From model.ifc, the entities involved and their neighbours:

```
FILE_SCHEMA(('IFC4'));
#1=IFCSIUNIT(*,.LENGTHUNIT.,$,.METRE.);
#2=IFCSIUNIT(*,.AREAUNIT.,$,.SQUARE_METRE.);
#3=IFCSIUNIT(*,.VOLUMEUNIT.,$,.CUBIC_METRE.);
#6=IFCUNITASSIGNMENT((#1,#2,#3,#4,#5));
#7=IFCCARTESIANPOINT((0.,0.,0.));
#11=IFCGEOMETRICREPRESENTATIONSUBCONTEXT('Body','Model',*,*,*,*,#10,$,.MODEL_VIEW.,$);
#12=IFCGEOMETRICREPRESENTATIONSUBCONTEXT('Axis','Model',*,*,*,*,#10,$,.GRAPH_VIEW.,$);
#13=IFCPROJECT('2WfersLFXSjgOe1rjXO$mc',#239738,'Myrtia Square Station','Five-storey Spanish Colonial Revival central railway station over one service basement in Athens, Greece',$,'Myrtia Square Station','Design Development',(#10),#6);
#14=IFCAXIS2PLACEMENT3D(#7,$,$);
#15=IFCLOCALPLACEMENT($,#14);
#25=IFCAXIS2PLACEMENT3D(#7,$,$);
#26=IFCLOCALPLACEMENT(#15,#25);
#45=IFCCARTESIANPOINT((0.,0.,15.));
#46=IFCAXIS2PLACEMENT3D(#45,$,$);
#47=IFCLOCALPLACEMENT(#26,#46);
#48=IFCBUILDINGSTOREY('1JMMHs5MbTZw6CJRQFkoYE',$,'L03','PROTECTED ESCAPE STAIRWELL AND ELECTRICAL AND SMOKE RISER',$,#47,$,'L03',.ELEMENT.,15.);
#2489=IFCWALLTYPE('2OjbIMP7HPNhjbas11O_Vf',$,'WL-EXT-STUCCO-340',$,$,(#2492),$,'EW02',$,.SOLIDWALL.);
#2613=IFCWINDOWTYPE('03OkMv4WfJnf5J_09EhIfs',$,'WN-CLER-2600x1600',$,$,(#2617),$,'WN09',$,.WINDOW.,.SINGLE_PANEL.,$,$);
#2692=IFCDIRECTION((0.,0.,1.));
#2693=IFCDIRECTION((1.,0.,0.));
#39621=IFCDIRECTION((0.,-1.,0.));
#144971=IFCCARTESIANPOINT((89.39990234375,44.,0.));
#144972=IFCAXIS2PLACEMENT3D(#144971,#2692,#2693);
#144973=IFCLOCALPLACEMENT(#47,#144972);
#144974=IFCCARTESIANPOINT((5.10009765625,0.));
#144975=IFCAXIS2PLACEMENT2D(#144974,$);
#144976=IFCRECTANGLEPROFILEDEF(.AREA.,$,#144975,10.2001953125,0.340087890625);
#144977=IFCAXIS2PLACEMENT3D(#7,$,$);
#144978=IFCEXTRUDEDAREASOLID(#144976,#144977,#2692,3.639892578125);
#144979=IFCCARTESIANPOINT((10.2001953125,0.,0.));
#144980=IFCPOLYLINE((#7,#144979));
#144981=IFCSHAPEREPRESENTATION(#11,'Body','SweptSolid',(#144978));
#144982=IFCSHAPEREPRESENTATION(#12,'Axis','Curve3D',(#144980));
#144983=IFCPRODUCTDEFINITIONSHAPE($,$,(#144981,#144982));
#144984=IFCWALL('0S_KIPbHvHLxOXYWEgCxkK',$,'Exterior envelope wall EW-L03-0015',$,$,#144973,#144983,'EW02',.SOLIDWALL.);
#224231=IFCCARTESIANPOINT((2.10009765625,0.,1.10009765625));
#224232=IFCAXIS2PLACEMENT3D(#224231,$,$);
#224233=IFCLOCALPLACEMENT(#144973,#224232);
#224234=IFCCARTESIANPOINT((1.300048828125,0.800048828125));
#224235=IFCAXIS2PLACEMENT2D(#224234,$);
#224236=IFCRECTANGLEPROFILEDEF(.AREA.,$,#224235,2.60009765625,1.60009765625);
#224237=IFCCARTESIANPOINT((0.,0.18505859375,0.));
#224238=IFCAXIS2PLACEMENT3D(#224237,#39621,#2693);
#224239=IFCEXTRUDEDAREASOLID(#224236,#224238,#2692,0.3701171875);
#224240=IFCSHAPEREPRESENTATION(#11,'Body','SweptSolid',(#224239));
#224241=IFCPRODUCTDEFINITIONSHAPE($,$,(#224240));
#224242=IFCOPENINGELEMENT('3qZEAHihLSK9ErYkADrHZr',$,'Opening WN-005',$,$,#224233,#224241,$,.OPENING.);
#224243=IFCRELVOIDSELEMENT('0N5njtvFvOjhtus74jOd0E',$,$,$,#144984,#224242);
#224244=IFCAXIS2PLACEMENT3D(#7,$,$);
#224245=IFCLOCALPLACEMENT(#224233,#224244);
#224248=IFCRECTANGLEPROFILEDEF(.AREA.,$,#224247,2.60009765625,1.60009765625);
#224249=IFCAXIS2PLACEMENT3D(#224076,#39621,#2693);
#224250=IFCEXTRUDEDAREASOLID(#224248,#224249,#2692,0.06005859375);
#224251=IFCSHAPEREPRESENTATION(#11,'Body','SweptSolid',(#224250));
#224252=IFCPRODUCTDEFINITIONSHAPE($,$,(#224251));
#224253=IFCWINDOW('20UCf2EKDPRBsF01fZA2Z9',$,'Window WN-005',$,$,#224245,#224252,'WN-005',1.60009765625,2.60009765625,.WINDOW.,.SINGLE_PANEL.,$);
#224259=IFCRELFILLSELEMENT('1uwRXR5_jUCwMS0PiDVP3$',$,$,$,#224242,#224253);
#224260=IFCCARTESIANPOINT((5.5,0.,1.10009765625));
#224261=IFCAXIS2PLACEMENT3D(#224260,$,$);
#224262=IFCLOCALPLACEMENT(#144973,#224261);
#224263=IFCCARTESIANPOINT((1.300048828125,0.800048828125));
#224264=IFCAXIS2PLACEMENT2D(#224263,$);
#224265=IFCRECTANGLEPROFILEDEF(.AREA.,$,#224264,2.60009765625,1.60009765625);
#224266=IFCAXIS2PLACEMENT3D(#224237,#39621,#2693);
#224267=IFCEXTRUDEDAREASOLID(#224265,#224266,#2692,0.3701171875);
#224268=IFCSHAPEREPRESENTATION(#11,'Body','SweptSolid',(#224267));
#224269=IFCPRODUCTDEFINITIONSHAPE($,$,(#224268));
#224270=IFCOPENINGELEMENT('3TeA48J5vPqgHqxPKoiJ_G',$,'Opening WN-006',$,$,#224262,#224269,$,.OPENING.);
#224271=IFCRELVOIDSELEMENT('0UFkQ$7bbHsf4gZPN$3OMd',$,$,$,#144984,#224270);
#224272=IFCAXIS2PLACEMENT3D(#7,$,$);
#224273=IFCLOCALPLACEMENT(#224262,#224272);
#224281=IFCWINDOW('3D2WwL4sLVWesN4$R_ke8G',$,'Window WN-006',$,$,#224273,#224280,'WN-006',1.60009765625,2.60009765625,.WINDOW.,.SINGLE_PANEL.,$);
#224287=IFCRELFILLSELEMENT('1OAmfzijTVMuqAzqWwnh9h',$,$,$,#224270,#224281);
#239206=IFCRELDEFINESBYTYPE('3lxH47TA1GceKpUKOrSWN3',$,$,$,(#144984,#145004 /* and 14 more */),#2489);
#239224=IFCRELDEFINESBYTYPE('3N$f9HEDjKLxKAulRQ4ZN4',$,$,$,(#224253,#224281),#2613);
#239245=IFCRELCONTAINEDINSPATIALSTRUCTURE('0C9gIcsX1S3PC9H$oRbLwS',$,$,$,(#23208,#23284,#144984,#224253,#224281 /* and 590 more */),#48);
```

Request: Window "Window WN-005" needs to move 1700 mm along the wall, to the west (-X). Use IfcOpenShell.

```python
import ifcopenshell
import ifcopenshell.api.geometry
import ifcopenshell.util.placement
import ifcopenshell.util.unit

model = ifcopenshell.open("model.ifc")
unit_scale = ifcopenshell.util.unit.calculate_unit_scale(model)

window = model.by_id(224253)
opening = window.FillsVoids[0].RelatingOpeningElement
wall = opening.VoidsElements[0].RelatingBuildingElement

wall_matrix = ifcopenshell.util.placement.get_local_placement(wall.ObjectPlacement)
shift = wall_matrix[:3, 0] * -1.7 / unit_scale
before = ifcopenshell.util.placement.get_local_placement(window.ObjectPlacement)[:3, 3].copy()

# The window is placed relative to its opening, so it follows when the opening moves.
matrix = ifcopenshell.util.placement.get_local_placement(opening.ObjectPlacement)
matrix[:3, 3] += shift
ifcopenshell.api.geometry.edit_object_placement(
    model, product=opening, matrix=matrix, is_si=False, should_transform_children=True
)

after = ifcopenshell.util.placement.get_local_placement(window.ObjectPlacement)[:3, 3]
print("window moved by", (after - before).round(3) + 0.0)

model.write("model_rev.ifc")
```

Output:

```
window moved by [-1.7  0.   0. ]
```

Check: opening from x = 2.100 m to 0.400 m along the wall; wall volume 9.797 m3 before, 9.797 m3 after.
